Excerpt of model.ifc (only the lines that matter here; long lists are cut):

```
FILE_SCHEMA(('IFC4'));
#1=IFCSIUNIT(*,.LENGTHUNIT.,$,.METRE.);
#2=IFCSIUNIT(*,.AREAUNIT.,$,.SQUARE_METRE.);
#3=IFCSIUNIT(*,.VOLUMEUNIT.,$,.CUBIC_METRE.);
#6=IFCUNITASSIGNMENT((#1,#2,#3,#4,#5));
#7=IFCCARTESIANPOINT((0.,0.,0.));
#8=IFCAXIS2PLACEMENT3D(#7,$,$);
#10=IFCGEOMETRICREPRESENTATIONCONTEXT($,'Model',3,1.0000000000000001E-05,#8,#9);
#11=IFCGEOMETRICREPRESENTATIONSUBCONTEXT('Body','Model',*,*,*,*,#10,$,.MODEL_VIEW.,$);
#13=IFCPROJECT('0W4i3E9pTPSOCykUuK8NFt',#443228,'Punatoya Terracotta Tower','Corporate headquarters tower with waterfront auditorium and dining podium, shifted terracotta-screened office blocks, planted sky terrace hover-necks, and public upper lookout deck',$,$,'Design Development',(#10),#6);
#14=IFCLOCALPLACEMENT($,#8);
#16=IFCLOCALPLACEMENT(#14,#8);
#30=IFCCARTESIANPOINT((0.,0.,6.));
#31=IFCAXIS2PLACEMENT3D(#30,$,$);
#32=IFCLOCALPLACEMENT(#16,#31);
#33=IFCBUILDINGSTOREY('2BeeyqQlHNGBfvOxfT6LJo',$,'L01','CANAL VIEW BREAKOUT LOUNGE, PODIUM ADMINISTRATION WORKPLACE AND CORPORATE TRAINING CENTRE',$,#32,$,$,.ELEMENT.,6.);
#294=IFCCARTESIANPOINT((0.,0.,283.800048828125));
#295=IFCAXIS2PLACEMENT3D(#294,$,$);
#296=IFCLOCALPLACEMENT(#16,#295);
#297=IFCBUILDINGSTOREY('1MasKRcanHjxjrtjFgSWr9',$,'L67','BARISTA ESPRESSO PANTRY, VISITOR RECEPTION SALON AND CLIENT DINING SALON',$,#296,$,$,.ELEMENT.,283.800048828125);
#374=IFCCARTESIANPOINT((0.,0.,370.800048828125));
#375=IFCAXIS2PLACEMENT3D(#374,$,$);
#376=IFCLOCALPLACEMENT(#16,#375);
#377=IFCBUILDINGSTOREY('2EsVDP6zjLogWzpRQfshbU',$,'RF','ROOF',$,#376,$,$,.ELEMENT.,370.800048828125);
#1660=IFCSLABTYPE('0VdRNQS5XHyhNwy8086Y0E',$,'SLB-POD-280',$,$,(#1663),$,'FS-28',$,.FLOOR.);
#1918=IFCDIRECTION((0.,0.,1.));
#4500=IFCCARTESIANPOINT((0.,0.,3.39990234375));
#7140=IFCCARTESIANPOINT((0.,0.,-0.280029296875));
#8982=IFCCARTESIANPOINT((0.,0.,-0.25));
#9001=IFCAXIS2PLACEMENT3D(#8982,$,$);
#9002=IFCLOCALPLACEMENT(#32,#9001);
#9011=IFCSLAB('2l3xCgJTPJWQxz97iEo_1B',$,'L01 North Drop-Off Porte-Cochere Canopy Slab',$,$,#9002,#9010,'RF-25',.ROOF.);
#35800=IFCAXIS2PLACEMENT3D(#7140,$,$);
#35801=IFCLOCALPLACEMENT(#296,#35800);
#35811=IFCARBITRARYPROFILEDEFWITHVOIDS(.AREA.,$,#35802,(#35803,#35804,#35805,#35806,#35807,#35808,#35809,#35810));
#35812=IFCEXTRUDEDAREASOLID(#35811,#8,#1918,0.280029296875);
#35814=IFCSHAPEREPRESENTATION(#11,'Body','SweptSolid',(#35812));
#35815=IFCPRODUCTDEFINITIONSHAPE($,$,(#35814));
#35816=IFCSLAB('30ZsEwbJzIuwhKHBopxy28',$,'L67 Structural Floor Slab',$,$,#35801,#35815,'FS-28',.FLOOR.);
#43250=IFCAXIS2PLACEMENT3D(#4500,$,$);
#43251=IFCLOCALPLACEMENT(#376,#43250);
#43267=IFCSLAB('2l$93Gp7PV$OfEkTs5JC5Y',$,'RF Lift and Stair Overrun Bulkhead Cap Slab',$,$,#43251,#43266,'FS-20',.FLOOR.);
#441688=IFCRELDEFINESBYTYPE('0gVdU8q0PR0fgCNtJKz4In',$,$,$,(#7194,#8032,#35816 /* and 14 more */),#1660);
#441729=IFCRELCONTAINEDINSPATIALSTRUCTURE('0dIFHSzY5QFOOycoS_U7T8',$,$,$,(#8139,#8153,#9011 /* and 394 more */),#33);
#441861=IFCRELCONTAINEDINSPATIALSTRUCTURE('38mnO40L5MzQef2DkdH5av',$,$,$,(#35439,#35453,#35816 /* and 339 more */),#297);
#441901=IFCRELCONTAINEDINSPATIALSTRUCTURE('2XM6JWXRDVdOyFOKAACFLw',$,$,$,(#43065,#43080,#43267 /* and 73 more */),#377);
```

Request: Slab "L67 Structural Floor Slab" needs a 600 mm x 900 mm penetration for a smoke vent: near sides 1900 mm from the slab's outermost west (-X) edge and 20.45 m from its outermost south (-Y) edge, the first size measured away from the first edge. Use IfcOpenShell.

```python
import numpy as np
import ifcopenshell
import ifcopenshell.api.feature
import ifcopenshell.api.geometry
import ifcopenshell.api.root
import ifcopenshell.geom
import ifcopenshell.util.placement
import ifcopenshell.util.representation
import ifcopenshell.util.shape
import ifcopenshell.util.unit

model = ifcopenshell.open("model.ifc")
unit_scale = ifcopenshell.util.unit.calculate_unit_scale(model)
settings = ifcopenshell.geom.settings()


def volume(element):
    """Net volume in cubic metres, openings subtracted."""
    shape = ifcopenshell.geom.create_shape(settings, element)
    return ifcopenshell.util.shape.get_volume(shape.geometry)


slab = model.by_id(35816)
before = volume(slab)

# Extent in the slab's own axes, in metres. The edges named are its -X and -Y sides.
slab_shape = ifcopenshell.geom.create_shape(settings, slab)
vertices = ifcopenshell.util.shape.get_vertices(slab_shape.geometry)
x_min, y_min, bottom = vertices.min(axis=0)
top = vertices[:, 2].max()

opening = ifcopenshell.api.root.create_entity(model, ifc_class="IfcOpeningElement", name="Smoke vent opening", predefined_type="OPENING")
context = ifcopenshell.util.representation.get_context(model, "Model", "Body", "MODEL_VIEW")
width, depth = 0.6, 0.9
outline = [(0.0, 0.0), (width, 0.0), (width, depth), (0.0, depth), (0.0, 0.0)]
# Overshoot both faces by 50 mm so the cut is clean.
shape = ifcopenshell.api.geometry.add_slab_representation(
    model, context=context, depth=top - bottom + 0.1, polyline=outline
)
ifcopenshell.api.geometry.assign_representation(model, product=opening, representation=shape)

matrix = ifcopenshell.util.placement.get_local_placement(slab.ObjectPlacement)
matrix[:, 3] = matrix @ np.append(np.array([x_min + 1.9, y_min + 20.45, bottom - 0.05]) / unit_scale, 1.0)
ifcopenshell.api.geometry.edit_object_placement(model, product=opening, matrix=matrix, is_si=False)
ifcopenshell.api.feature.add_feature(model, feature=opening, element=slab)

after = volume(slab)

print(f"slab volume {before:.3f} -> {after:.3f} m3")

model.write("model_v2.ifc")
```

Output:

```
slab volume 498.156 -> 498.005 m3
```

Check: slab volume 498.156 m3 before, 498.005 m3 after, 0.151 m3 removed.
